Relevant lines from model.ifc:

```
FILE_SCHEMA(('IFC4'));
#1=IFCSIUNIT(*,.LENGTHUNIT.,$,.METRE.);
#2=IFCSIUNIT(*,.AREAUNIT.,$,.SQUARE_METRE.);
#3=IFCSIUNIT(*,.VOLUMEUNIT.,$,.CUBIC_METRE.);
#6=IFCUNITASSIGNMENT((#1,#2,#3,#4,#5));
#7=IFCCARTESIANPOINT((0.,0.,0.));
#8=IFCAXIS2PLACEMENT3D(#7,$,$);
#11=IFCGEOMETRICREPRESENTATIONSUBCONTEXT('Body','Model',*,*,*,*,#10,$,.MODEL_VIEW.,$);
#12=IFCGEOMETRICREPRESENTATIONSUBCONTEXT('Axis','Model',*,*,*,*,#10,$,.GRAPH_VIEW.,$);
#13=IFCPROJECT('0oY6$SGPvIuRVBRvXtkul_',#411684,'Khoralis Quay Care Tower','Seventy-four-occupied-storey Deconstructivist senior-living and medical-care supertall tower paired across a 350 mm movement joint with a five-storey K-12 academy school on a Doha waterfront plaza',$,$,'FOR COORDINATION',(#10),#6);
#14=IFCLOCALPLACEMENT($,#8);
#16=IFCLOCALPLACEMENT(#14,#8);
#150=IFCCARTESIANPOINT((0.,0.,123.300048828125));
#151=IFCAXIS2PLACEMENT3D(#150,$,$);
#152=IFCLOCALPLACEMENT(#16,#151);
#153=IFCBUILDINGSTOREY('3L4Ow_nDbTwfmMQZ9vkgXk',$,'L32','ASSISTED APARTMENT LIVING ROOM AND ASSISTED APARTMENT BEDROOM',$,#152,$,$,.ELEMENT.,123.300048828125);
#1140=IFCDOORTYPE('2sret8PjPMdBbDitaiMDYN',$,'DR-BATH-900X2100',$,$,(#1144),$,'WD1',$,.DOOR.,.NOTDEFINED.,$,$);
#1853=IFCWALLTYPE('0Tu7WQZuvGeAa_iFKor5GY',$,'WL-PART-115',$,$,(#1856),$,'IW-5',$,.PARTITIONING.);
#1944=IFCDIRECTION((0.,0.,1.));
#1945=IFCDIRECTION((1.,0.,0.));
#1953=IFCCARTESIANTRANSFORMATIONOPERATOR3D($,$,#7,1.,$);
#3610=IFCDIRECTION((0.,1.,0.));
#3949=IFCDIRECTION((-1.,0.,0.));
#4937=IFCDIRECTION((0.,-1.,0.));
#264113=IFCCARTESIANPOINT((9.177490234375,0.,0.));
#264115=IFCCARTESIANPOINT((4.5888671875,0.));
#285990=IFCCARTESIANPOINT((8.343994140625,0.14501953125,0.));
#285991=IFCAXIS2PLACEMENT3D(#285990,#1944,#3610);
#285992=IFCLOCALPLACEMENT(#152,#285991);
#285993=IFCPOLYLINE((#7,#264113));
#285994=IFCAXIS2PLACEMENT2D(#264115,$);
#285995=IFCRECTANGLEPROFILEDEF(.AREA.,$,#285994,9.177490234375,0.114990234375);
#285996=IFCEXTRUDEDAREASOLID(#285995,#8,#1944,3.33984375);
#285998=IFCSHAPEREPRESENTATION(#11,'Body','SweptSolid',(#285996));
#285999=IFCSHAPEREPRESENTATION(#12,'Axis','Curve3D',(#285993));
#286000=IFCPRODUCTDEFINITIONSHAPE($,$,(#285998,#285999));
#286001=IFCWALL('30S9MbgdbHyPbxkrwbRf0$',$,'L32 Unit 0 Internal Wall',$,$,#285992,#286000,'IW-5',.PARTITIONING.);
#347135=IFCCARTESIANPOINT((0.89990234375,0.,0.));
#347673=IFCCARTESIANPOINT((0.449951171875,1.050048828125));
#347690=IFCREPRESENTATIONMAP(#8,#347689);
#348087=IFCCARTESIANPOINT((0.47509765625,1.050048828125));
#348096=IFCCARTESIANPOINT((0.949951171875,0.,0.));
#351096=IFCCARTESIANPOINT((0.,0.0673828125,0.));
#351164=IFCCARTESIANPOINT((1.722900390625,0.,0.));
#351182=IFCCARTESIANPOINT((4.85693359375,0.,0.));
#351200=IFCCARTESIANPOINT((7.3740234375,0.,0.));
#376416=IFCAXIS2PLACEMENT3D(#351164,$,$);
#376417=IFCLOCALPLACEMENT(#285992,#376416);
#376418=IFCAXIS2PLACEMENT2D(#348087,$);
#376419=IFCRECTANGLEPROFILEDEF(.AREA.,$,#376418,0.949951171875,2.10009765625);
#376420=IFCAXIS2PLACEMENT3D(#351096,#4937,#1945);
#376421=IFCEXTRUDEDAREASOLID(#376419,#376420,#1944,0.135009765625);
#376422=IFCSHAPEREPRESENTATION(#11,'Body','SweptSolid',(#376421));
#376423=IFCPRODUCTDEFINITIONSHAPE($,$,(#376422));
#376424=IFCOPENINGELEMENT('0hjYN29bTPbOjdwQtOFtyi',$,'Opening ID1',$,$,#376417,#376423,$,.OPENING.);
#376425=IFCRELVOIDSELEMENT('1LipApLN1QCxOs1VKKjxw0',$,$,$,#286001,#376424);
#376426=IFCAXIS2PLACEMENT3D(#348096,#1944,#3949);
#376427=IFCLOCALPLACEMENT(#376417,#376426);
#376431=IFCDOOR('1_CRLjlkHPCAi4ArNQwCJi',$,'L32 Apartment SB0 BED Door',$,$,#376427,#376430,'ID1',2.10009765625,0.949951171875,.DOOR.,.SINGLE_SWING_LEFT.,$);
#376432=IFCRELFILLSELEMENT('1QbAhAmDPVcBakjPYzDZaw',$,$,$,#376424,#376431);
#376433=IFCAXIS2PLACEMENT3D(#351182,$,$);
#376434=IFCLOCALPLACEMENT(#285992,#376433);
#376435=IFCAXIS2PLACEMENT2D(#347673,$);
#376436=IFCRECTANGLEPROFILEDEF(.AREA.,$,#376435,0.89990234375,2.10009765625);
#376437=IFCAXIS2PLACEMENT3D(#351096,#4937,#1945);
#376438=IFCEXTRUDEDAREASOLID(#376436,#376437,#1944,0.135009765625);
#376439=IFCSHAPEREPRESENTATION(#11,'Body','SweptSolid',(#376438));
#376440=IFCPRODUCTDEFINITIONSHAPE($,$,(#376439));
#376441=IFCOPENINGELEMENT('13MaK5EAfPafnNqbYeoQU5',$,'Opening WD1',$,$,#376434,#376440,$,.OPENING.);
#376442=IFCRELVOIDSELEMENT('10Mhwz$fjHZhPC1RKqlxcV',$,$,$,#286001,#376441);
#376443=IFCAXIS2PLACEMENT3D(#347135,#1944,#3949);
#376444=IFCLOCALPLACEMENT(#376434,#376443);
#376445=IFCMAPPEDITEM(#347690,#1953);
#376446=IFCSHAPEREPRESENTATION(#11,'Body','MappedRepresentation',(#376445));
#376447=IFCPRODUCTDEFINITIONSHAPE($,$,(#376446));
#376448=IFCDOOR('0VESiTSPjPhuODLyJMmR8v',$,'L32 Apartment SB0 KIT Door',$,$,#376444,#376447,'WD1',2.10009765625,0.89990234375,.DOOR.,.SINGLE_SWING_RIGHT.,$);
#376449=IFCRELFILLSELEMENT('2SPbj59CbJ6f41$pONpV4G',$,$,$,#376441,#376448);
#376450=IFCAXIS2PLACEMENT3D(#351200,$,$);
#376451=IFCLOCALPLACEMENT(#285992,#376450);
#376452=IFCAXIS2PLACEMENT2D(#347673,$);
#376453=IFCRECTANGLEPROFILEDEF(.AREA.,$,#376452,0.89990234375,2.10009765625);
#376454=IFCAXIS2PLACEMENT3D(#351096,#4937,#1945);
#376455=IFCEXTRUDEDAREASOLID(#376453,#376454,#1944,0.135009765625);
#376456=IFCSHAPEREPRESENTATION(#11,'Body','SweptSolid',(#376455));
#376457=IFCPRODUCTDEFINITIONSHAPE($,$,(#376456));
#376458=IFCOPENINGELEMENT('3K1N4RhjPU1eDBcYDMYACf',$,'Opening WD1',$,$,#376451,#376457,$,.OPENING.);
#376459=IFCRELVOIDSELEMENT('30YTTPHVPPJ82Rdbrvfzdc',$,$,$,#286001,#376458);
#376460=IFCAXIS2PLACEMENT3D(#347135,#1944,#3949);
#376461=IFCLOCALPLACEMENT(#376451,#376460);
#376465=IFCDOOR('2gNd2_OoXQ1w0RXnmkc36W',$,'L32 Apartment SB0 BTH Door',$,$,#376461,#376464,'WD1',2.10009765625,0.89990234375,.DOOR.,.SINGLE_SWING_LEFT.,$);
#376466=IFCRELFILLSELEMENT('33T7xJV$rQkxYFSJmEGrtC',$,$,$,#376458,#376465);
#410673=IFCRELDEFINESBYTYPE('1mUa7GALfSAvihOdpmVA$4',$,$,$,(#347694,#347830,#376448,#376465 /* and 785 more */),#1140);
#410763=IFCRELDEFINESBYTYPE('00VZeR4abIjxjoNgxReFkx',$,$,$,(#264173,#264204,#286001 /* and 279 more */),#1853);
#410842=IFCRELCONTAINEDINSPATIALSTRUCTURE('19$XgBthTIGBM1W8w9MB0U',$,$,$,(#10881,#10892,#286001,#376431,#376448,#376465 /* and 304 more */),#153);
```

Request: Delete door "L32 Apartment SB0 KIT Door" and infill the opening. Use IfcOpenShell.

```python
import ifcopenshell
import ifcopenshell.api.feature
import ifcopenshell.api.root
import ifcopenshell.geom
import ifcopenshell.util.shape

model = ifcopenshell.open("model.ifc")
settings = ifcopenshell.geom.settings()


def volume(element):
    """Net volume in cubic metres, openings subtracted."""
    shape = ifcopenshell.geom.create_shape(settings, element)
    return ifcopenshell.util.shape.get_volume(shape.geometry)


door = model.by_guid("0VESiTSPjPhuODLyJMmR8v")
opening = door.FillsVoids[0].RelatingOpeningElement
wall = opening.VoidsElements[0].RelatingBuildingElement
before = volume(wall)

ifcopenshell.api.root.remove_product(model, product=door)
ifcopenshell.api.feature.remove_feature(model, feature=opening)

after = volume(wall)

print(f"wall volume {before:.3f} -> {after:.3f} m3")

model.write("model_edited.ifc")
```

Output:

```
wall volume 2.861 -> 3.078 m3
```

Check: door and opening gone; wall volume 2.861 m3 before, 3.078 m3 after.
